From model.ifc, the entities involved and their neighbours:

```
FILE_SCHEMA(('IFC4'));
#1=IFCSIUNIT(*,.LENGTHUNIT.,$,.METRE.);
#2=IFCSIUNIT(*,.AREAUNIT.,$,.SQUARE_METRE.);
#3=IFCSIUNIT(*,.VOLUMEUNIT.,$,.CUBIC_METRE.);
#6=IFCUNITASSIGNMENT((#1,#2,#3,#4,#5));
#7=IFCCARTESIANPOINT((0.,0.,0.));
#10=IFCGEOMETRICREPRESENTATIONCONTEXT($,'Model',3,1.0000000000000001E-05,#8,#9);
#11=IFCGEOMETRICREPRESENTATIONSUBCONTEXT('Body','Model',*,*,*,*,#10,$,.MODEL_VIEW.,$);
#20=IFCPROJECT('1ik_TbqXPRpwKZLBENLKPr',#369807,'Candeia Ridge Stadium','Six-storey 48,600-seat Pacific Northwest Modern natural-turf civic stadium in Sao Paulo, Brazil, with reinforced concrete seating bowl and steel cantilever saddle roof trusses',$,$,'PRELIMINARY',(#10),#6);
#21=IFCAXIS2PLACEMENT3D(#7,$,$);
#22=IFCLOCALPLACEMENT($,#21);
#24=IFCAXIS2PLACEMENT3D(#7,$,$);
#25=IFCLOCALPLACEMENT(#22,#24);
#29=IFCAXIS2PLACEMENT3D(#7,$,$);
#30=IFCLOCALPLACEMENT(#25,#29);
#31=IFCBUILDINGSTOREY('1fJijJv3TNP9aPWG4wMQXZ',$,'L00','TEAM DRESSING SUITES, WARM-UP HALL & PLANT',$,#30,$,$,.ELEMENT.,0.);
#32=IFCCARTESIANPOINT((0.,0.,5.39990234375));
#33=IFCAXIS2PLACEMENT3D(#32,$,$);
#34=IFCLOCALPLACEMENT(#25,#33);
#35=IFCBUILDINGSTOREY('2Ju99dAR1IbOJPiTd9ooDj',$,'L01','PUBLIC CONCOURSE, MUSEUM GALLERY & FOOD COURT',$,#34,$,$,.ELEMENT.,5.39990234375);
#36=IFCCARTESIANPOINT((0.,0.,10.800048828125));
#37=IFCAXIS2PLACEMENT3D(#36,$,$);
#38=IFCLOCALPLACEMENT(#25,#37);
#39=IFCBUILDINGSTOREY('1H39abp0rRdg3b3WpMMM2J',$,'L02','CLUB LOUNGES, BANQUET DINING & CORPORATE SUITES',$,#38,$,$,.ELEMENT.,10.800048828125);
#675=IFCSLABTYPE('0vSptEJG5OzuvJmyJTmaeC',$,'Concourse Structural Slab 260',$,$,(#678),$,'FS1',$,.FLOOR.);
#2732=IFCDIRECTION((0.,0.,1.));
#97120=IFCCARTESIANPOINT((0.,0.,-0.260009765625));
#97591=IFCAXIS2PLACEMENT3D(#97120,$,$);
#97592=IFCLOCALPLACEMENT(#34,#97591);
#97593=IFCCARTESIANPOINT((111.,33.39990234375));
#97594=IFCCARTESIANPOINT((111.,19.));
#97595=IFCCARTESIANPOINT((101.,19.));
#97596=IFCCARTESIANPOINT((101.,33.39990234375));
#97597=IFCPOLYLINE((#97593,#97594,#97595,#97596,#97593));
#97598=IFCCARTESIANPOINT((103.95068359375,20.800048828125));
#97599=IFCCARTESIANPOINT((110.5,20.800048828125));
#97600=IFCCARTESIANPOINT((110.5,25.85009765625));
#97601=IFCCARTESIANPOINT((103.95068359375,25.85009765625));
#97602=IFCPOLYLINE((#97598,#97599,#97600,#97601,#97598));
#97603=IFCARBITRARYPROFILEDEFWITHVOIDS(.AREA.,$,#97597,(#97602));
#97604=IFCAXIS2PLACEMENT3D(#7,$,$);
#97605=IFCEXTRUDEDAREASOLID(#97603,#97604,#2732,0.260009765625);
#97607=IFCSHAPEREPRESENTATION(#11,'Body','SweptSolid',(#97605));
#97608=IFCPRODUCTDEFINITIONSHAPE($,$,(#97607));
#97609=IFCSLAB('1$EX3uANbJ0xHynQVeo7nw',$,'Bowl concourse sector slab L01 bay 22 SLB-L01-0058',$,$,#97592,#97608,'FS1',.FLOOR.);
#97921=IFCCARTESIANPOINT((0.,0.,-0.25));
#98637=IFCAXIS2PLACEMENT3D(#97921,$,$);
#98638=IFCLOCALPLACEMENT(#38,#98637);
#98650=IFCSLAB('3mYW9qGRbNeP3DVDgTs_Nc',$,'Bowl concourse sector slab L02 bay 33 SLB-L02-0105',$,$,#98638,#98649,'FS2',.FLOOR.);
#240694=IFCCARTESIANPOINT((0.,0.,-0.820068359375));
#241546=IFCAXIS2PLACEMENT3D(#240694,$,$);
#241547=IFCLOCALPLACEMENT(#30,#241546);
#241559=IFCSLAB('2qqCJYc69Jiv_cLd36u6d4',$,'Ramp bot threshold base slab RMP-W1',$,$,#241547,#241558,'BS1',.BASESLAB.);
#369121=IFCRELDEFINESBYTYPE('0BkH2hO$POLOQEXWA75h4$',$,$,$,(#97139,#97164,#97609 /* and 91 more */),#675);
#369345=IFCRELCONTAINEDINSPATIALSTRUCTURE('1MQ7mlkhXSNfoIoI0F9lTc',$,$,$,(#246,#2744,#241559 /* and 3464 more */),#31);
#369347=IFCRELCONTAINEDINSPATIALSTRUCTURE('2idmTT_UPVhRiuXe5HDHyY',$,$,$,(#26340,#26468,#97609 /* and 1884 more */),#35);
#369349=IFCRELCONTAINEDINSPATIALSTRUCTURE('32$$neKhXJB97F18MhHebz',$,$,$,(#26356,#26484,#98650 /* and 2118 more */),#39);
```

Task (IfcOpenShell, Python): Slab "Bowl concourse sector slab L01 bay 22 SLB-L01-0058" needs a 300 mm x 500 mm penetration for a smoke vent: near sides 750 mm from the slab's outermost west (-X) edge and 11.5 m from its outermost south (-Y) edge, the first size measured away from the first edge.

```python
import numpy as np
import ifcopenshell
import ifcopenshell.api.feature
import ifcopenshell.api.geometry
import ifcopenshell.api.root
import ifcopenshell.geom
import ifcopenshell.util.placement
import ifcopenshell.util.representation
import ifcopenshell.util.shape
import ifcopenshell.util.unit

model = ifcopenshell.open("model.ifc")
unit_scale = ifcopenshell.util.unit.calculate_unit_scale(model)
settings = ifcopenshell.geom.settings()


def volume(element):
    """Net volume in cubic metres, openings subtracted."""
    shape = ifcopenshell.geom.create_shape(settings, element)
    return ifcopenshell.util.shape.get_volume(shape.geometry)


slab = model.by_id(97609)
before = volume(slab)

# Extent in the slab's own axes, in metres. The edges named are its -X and -Y sides.
slab_shape = ifcopenshell.geom.create_shape(settings, slab)
vertices = ifcopenshell.util.shape.get_vertices(slab_shape.geometry)
x_min, y_min, bottom = vertices.min(axis=0)
top = vertices[:, 2].max()

opening = ifcopenshell.api.root.create_entity(model, ifc_class="IfcOpeningElement", name="Smoke vent opening", predefined_type="OPENING")
context = ifcopenshell.util.representation.get_context(model, "Model", "Body", "MODEL_VIEW")
width, depth = 0.3, 0.5
outline = [(0.0, 0.0), (width, 0.0), (width, depth), (0.0, depth), (0.0, 0.0)]
# Overshoot both faces by 50 mm so the cut is clean.
shape = ifcopenshell.api.geometry.add_slab_representation(
    model, context=context, depth=top - bottom + 0.1, polyline=outline
)
ifcopenshell.api.geometry.assign_representation(model, product=opening, representation=shape)

matrix = ifcopenshell.util.placement.get_local_placement(slab.ObjectPlacement)
matrix[:, 3] = matrix @ np.append(np.array([x_min + 0.75, y_min + 11.5, bottom - 0.05]) / unit_scale, 1.0)
ifcopenshell.api.geometry.edit_object_placement(model, product=opening, matrix=matrix, is_si=False)
ifcopenshell.api.feature.add_feature(model, feature=opening, element=slab)

after = volume(slab)

print(f"slab volume {before:.3f} -> {after:.3f} m3")

model.write("model_edited.ifc")
```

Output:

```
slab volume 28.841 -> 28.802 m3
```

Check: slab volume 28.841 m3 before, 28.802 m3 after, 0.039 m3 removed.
